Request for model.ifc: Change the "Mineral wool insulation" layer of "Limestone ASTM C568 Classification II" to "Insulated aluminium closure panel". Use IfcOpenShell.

First a look at what the model holds.

```python
import ifcopenshell
import ifcopenshell.util.element

model = ifcopenshell.open("model.ifc")
print(model.schema)
for layer_set in model.by_type("IfcMaterialLayerSet"):
    if layer_set.LayerSetName == "Limestone ASTM C568 Classification II":
        for layer in layer_set.MaterialLayers:
            print(layer.id(), layer.Material and layer.Material.Name, layer.LayerThickness, sep=" | ")
        print(len(ifcopenshell.util.element.get_elements_by_material(model, layer_set)), "elements and types use it")
print(sorted(m.Name for m in model.by_type("IfcMaterial") if m.Name)[:60])
```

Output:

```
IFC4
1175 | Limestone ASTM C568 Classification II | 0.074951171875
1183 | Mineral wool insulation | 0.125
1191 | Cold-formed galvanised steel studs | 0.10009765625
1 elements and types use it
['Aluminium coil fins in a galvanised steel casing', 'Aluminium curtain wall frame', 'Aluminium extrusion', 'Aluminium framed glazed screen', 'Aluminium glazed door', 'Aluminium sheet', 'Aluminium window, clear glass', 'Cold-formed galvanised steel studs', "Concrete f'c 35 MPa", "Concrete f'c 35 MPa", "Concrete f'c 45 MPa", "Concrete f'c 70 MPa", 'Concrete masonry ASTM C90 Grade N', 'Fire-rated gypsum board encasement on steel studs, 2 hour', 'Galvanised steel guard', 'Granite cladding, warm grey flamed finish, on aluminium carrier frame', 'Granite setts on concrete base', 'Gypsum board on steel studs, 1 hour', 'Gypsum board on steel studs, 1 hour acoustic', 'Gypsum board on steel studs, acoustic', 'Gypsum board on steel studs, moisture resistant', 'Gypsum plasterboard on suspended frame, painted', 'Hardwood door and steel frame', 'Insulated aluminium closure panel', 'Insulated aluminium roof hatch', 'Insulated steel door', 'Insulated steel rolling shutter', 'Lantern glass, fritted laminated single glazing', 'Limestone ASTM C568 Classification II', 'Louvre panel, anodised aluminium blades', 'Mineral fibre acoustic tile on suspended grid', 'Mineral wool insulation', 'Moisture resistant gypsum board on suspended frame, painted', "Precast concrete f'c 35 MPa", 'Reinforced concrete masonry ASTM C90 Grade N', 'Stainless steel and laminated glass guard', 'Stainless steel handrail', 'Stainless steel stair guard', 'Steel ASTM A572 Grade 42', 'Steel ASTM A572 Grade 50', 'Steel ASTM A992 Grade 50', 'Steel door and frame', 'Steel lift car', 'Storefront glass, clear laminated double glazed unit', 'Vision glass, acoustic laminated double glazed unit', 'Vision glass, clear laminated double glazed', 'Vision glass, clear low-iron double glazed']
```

```python
import ifcopenshell
import ifcopenshell.api.material

model = ifcopenshell.open("model.ifc")

layer_set = next(s for s in model.by_type("IfcMaterialLayerSet") if s.LayerSetName == "Limestone ASTM C568 Classification II")
layer = next(l for l in layer_set.MaterialLayers if l.Material and l.Material.Name == "Mineral wool insulation")
material = next(m for m in model.by_type("IfcMaterial") if m.Name == "Insulated aluminium closure panel")

# Point this one layer at the other material; renaming the old one would change it everywhere.
ifcopenshell.api.material.edit_layer(model, layer=layer, attributes={}, material=material)

print([l.Material.Name if l.Material else None for l in layer_set.MaterialLayers])

model.write("model_v2.ifc")
```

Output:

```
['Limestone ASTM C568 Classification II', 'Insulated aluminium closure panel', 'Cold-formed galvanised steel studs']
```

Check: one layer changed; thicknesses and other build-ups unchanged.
